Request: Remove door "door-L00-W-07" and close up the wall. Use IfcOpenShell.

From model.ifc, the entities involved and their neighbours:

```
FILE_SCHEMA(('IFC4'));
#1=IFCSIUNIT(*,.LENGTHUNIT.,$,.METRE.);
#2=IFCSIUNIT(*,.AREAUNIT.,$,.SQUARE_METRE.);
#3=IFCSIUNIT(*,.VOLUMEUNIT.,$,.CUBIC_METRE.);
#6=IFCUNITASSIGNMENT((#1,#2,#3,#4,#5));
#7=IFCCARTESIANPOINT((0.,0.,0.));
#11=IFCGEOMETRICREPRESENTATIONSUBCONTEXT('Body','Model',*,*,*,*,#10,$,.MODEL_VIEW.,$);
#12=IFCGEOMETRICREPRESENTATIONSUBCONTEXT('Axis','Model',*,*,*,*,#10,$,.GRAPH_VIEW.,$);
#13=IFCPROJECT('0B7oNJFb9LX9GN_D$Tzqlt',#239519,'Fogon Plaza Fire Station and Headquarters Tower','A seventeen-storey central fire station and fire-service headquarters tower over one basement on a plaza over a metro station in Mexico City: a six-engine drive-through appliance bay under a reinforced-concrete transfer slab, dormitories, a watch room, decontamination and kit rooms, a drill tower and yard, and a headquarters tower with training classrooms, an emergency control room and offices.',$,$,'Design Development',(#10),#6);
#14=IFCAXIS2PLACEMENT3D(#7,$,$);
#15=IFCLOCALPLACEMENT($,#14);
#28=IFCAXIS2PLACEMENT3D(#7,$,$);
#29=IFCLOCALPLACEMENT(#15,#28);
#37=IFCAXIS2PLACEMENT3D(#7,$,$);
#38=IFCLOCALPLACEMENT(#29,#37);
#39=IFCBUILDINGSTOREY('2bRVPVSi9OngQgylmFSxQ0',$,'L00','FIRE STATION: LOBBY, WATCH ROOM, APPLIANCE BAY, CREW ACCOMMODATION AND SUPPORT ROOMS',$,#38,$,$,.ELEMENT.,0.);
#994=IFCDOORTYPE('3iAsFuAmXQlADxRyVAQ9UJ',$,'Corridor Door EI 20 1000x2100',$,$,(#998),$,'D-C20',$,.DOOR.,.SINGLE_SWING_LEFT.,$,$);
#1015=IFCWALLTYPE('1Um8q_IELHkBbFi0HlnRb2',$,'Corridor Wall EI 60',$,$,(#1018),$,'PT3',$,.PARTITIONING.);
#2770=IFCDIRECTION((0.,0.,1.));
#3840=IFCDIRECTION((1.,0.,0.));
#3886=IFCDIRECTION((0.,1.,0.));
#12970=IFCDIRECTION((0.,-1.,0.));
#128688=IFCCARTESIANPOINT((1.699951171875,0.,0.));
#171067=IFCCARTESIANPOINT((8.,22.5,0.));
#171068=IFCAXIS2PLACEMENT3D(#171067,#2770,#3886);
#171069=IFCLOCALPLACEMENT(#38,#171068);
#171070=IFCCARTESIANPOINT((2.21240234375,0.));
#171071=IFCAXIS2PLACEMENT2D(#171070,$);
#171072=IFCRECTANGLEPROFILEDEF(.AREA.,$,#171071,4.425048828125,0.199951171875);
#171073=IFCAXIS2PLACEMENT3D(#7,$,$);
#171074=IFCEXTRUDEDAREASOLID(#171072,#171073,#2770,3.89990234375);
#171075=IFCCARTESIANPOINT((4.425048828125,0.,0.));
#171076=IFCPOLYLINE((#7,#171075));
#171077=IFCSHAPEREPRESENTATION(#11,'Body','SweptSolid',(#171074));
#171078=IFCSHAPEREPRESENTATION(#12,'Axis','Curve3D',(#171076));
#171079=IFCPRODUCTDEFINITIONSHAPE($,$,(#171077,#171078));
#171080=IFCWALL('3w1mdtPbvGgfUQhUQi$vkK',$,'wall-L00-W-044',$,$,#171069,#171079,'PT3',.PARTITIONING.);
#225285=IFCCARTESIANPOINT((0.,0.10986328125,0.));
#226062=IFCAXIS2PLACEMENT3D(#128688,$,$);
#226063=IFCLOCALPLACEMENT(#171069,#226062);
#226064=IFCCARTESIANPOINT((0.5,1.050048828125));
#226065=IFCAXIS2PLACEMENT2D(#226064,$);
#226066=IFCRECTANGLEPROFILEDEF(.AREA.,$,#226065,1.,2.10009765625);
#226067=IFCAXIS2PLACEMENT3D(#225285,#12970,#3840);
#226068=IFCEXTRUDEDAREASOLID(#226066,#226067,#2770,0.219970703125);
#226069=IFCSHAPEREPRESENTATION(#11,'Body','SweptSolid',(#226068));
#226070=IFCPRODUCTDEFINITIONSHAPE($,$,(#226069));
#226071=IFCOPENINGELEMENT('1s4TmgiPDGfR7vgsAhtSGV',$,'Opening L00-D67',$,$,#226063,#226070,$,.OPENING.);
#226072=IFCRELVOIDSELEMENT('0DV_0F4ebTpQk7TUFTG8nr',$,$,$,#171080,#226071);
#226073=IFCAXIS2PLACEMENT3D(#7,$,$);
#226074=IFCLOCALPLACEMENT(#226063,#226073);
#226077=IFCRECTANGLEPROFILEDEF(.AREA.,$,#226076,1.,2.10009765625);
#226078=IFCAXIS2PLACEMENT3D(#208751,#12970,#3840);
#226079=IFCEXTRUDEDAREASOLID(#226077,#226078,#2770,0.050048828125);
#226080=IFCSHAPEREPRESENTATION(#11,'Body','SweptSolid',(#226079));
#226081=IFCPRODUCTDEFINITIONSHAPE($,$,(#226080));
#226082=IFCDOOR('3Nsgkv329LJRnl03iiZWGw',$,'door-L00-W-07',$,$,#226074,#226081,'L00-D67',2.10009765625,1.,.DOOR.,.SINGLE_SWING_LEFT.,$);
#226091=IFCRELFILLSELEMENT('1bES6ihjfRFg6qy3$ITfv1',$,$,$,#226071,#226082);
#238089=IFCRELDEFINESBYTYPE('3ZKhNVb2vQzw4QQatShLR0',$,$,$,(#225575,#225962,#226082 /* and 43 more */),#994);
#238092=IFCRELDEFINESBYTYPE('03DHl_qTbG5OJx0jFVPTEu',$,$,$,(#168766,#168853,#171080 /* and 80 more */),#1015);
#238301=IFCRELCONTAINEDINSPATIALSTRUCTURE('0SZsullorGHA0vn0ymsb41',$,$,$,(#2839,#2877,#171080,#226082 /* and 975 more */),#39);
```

```python
import ifcopenshell
import ifcopenshell.api.feature
import ifcopenshell.api.root
import ifcopenshell.geom
import ifcopenshell.util.shape

model = ifcopenshell.open("model.ifc")
settings = ifcopenshell.geom.settings()


def volume(element):
    """Net volume in cubic metres, openings subtracted."""
    shape = ifcopenshell.geom.create_shape(settings, element)
    return ifcopenshell.util.shape.get_volume(shape.geometry)


door = model.by_guid("3Nsgkv329LJRnl03iiZWGw")
opening = door.FillsVoids[0].RelatingOpeningElement
wall = opening.VoidsElements[0].RelatingBuildingElement
before = volume(wall)

ifcopenshell.api.root.remove_product(model, product=door)
ifcopenshell.api.feature.remove_feature(model, feature=opening)

after = volume(wall)

print(f"wall volume {before:.3f} -> {after:.3f} m3")

model.write("model_edited.ifc")
```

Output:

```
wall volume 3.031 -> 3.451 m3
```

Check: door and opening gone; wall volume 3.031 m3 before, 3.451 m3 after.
